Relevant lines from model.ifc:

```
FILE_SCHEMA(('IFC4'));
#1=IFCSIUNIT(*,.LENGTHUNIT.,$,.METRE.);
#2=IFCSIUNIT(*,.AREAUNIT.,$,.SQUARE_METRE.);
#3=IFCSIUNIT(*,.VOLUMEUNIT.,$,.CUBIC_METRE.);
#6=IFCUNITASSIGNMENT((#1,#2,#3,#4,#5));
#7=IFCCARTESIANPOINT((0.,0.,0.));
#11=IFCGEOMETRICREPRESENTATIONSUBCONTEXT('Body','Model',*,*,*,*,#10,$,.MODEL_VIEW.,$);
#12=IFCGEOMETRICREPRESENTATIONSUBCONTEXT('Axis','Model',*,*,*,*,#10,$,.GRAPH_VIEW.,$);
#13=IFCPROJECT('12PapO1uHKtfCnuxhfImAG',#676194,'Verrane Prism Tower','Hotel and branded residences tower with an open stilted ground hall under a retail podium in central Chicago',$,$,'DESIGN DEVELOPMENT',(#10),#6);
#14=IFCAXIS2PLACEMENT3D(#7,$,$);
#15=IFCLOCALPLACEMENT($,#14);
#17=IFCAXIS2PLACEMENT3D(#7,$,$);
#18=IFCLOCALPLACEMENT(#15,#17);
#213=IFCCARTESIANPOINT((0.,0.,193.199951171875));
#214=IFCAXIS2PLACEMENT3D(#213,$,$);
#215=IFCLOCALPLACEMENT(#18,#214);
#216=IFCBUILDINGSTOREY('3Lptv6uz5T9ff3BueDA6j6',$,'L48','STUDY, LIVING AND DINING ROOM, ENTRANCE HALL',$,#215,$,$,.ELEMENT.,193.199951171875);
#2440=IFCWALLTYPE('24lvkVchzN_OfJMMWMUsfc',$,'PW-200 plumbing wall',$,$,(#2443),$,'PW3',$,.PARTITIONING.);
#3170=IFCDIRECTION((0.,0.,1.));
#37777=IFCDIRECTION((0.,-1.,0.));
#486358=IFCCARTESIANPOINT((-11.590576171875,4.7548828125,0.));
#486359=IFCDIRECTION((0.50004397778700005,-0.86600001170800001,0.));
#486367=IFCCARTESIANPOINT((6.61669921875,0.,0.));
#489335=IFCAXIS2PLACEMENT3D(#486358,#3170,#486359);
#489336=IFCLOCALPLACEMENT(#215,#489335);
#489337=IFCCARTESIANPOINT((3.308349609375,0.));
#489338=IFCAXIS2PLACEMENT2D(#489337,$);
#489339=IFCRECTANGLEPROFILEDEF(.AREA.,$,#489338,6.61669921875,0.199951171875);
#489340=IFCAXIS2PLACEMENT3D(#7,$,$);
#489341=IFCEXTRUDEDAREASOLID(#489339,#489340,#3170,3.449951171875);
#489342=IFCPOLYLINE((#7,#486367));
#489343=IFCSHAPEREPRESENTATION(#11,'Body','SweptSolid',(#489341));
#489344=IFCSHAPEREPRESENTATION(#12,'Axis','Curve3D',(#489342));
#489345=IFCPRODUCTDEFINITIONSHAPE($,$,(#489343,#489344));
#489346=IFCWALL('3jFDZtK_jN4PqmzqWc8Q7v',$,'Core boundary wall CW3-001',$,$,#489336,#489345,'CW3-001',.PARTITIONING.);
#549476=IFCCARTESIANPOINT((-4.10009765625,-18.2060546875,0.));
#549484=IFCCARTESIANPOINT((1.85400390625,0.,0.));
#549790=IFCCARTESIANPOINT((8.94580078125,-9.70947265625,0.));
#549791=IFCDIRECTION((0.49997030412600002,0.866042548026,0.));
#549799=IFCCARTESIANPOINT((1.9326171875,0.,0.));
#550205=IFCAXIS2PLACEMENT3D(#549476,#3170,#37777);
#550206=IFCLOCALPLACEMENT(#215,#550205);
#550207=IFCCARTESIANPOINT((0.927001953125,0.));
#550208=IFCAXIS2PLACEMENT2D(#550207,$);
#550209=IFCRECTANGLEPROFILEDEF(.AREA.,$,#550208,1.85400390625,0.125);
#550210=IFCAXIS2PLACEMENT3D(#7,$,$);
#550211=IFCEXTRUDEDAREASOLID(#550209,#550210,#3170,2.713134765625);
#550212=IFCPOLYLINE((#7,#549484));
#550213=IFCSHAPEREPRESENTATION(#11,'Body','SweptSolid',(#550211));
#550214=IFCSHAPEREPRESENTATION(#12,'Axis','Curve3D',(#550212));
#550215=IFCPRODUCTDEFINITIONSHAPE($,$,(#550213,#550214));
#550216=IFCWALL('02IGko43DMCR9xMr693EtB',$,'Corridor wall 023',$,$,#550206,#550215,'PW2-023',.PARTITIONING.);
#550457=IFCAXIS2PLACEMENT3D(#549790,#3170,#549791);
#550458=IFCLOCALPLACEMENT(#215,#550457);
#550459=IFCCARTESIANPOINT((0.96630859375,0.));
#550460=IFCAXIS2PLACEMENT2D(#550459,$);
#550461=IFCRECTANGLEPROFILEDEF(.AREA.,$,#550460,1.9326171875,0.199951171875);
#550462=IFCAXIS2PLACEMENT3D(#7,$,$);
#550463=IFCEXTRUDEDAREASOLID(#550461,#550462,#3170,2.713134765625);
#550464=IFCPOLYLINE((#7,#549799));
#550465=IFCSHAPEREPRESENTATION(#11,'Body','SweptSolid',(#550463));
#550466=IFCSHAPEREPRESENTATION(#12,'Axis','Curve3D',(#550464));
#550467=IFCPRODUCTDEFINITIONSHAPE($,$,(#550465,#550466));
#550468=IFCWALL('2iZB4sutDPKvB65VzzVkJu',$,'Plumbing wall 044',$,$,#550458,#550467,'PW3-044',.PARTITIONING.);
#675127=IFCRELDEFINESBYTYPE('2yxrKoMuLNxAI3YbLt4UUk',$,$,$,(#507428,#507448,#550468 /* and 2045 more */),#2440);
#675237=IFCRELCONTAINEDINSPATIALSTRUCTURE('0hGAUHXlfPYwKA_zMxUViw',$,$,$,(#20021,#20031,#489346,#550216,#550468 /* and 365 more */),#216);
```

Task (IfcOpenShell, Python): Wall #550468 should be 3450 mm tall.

```python
import ifcopenshell
import ifcopenshell.geom
import ifcopenshell.util.representation
import ifcopenshell.util.shape
import ifcopenshell.util.unit

model = ifcopenshell.open("model.ifc")
unit_scale = ifcopenshell.util.unit.calculate_unit_scale(model)
settings = ifcopenshell.geom.settings()


def volume(element):
    """Net volume in cubic metres, openings subtracted."""
    shape = ifcopenshell.geom.create_shape(settings, element)
    return ifcopenshell.util.shape.get_volume(shape.geometry)


wall = model.by_id(550468)
before = volume(wall)

body = ifcopenshell.util.representation.get_representation(wall, "Model", "Body")
solid = body.Items[0]
old_height = solid.Depth
solid.Depth = 3.45 / unit_scale
after = volume(wall)

print(f"height {old_height:g} -> {solid.Depth:g}, volume {before:.3f} -> {after:.3f} m3")

model.write("model_rev.ifc")
```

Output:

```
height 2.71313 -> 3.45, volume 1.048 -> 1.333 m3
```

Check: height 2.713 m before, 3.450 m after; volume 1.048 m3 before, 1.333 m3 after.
